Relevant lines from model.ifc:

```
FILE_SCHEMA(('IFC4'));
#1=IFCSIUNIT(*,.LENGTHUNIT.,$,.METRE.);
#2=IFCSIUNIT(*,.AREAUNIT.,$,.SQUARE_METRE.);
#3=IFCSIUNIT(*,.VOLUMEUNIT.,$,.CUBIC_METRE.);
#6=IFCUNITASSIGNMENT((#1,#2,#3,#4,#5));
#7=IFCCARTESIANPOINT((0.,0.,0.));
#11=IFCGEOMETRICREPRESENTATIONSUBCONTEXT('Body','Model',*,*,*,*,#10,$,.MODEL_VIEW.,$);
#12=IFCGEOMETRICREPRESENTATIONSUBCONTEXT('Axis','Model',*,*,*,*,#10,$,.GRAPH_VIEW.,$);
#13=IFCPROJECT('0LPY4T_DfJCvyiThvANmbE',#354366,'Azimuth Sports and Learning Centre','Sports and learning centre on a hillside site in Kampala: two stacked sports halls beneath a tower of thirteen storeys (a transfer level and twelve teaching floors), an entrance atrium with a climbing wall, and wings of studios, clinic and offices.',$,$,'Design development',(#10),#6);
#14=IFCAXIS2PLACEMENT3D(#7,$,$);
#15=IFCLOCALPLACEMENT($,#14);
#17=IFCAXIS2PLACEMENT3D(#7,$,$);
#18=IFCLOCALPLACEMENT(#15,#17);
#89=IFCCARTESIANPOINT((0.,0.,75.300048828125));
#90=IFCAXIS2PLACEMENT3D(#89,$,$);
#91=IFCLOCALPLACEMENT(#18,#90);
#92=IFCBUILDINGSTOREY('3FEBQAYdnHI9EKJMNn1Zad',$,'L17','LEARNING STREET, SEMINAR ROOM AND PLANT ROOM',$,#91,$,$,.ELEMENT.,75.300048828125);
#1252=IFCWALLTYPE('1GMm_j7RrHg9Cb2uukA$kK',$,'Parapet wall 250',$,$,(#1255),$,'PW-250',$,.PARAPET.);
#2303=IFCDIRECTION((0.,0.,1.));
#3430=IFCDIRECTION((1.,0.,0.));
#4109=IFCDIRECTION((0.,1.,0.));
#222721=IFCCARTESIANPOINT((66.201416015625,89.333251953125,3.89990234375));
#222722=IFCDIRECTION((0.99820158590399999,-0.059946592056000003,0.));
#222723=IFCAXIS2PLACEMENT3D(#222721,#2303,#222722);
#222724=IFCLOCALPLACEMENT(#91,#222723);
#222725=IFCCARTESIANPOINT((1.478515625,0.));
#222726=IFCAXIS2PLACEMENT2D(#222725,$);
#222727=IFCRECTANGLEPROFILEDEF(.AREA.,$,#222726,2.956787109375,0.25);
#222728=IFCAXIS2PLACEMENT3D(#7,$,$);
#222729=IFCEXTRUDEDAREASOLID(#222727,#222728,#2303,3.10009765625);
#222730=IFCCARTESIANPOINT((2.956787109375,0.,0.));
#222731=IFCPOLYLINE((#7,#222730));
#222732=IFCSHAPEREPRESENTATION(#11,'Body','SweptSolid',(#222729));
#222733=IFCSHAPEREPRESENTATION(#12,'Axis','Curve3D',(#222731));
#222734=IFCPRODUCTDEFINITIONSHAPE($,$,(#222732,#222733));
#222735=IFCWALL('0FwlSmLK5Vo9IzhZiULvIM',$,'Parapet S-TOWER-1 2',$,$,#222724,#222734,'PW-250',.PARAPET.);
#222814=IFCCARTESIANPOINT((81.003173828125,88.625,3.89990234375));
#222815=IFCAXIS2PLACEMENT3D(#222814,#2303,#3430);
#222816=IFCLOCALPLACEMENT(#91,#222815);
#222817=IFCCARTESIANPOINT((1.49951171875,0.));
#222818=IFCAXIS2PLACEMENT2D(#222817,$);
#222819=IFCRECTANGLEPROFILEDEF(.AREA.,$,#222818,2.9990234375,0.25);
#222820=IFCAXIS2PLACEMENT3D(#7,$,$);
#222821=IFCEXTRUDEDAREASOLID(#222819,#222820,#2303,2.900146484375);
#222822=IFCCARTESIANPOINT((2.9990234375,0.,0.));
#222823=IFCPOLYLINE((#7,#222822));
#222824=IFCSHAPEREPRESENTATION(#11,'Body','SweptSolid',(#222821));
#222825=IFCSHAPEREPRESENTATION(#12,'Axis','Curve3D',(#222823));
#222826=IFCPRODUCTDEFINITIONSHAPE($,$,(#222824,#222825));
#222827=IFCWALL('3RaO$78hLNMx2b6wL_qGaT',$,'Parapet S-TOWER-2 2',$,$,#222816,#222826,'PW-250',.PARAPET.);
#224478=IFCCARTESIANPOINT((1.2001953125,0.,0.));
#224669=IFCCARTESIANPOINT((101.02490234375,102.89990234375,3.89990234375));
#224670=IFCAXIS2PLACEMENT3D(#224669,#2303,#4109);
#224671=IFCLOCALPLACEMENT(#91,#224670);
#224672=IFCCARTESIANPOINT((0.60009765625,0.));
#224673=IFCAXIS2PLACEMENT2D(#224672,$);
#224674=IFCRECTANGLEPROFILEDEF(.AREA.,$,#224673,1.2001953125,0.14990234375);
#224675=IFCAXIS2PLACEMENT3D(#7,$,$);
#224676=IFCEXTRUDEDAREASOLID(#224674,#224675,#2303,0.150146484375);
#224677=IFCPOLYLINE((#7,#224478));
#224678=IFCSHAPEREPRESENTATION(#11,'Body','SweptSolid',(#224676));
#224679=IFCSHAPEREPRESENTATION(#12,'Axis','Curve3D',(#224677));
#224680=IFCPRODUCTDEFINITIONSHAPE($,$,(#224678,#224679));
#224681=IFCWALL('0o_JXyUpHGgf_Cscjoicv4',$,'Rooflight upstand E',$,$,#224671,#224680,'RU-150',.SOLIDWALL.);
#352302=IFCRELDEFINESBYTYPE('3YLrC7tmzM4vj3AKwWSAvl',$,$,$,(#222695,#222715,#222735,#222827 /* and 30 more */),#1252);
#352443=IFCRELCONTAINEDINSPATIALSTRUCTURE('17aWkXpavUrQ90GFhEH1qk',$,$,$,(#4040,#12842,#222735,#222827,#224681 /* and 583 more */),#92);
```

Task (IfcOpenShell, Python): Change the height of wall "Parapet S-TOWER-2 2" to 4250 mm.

```python
import ifcopenshell
import ifcopenshell.geom
import ifcopenshell.util.representation
import ifcopenshell.util.shape
import ifcopenshell.util.unit

model = ifcopenshell.open("model.ifc")
unit_scale = ifcopenshell.util.unit.calculate_unit_scale(model)
settings = ifcopenshell.geom.settings()


def volume(element):
    """Net volume in cubic metres, openings subtracted."""
    shape = ifcopenshell.geom.create_shape(settings, element)
    return ifcopenshell.util.shape.get_volume(shape.geometry)


wall = model.by_id(222827)
before = volume(wall)

body = ifcopenshell.util.representation.get_representation(wall, "Model", "Body")
solid = body.Items[0]
old_height = solid.Depth
solid.Depth = 4.25 / unit_scale
after = volume(wall)

print(f"height {old_height:g} -> {solid.Depth:g}, volume {before:.3f} -> {after:.3f} m3")

model.write("model_edited.ifc")
```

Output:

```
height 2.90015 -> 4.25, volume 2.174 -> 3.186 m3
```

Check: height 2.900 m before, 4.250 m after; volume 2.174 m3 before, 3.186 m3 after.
